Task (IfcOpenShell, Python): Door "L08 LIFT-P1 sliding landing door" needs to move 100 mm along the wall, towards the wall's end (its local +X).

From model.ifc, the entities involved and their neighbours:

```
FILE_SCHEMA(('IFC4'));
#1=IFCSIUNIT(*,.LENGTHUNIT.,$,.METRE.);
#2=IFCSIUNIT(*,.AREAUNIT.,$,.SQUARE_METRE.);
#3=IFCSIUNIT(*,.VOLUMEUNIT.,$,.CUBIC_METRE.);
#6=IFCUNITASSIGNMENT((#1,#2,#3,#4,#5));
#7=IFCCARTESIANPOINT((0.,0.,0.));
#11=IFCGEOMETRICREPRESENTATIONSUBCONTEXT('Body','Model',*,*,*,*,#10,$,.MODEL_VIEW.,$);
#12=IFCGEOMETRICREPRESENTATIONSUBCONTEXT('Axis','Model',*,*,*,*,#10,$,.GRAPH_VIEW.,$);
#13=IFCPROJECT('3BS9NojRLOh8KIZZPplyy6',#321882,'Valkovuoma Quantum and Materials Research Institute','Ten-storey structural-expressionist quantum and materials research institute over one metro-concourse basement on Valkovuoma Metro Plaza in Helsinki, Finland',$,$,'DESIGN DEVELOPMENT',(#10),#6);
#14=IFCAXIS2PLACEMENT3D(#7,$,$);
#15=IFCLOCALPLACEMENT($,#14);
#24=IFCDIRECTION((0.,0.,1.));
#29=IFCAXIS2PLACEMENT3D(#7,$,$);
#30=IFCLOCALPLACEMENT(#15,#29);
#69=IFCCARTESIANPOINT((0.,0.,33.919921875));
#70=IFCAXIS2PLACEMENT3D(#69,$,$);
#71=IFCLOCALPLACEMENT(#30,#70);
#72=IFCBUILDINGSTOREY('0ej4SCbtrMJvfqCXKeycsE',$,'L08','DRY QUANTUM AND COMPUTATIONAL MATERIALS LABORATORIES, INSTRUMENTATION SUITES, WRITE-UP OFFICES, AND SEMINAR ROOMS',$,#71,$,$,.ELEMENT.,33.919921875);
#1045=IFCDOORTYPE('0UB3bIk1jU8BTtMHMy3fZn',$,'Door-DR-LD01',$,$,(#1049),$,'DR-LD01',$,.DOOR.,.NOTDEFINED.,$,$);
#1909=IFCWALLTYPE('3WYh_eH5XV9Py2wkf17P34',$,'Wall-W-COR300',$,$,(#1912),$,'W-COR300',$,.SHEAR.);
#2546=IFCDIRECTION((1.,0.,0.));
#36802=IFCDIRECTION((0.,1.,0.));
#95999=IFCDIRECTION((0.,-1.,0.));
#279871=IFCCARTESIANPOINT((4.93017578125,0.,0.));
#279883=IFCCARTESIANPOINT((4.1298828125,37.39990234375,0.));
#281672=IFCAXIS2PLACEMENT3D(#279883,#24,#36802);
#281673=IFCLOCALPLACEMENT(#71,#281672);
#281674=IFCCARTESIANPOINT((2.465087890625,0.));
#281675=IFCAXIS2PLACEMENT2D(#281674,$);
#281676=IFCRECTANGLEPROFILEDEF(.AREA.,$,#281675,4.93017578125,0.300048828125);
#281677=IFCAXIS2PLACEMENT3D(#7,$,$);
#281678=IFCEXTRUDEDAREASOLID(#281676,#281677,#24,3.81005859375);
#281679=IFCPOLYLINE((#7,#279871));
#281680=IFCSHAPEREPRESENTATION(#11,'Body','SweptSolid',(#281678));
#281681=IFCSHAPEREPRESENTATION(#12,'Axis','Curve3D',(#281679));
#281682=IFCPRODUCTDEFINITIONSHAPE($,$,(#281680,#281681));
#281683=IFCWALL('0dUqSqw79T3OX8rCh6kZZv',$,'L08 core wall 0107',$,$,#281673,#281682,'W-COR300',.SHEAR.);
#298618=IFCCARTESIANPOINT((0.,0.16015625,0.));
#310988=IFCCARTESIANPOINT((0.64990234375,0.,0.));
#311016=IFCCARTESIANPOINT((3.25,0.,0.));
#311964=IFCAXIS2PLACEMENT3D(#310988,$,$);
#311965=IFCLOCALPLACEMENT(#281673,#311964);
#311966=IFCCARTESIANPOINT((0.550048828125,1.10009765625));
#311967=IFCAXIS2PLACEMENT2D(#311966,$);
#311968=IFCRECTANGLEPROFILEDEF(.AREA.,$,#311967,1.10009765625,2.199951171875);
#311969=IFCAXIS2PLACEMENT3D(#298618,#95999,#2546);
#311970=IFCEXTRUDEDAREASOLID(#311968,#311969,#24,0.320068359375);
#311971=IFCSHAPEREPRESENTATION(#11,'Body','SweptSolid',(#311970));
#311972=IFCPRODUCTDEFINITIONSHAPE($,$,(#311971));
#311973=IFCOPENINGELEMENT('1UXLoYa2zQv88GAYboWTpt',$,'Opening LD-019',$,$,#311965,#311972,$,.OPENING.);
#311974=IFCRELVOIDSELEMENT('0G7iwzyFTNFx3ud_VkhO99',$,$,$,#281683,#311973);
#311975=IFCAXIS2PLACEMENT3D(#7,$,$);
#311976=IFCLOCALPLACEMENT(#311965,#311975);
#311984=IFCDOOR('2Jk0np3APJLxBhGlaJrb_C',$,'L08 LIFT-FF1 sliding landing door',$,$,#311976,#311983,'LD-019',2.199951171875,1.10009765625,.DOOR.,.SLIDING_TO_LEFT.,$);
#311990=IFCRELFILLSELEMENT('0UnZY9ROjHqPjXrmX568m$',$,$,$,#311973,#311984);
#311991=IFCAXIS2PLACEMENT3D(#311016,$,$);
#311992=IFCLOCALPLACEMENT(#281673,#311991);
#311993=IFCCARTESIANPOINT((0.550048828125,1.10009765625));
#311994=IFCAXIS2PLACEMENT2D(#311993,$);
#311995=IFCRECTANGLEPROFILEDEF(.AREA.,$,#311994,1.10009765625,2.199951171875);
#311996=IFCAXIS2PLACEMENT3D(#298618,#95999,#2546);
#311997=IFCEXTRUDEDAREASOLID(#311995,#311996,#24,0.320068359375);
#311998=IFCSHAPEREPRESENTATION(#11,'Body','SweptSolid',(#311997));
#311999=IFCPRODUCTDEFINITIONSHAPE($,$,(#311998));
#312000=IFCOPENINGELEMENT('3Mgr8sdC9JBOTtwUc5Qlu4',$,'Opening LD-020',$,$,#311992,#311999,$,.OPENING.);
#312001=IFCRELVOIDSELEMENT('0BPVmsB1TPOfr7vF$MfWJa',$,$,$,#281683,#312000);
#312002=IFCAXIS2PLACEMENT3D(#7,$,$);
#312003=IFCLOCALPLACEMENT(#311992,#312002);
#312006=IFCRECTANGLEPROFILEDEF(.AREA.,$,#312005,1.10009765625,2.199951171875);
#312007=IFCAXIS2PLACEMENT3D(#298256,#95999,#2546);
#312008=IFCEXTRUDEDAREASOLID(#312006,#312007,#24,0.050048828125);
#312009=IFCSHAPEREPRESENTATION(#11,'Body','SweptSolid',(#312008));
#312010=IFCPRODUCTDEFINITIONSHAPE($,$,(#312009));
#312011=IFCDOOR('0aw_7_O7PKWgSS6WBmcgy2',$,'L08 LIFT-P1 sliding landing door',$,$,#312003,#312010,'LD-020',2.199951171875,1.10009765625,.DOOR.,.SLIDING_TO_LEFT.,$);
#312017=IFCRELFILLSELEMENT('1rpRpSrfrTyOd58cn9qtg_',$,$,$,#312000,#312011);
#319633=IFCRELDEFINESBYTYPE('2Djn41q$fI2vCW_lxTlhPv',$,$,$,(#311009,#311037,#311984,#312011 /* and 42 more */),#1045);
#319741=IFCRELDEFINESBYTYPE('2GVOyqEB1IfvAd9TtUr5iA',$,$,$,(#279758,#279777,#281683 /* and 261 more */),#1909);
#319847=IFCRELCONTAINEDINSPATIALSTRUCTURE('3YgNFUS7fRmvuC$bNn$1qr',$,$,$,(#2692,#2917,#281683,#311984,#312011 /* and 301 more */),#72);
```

```python
import ifcopenshell
import ifcopenshell.api.geometry
import ifcopenshell.util.placement

model = ifcopenshell.open("model.ifc")

door = model.by_guid("0aw_7_O7PKWgSS6WBmcgy2")
opening = door.FillsVoids[0].RelatingOpeningElement
wall = opening.VoidsElements[0].RelatingBuildingElement

wall_matrix = ifcopenshell.util.placement.get_local_placement(wall.ObjectPlacement)
shift = wall_matrix[:3, 0] * 0.1
before = ifcopenshell.util.placement.get_local_placement(door.ObjectPlacement)[:3, 3].copy()

# The door is placed relative to its opening, so it follows when the opening moves.
matrix = ifcopenshell.util.placement.get_local_placement(opening.ObjectPlacement)
matrix[:3, 3] += shift
ifcopenshell.api.geometry.edit_object_placement(
    model, product=opening, matrix=matrix, is_si=False, should_transform_children=True
)

after = ifcopenshell.util.placement.get_local_placement(door.ObjectPlacement)[:3, 3]
print("door moved by", (after - before).round(3) + 0.0)

model.write("model_updated.ifc")
```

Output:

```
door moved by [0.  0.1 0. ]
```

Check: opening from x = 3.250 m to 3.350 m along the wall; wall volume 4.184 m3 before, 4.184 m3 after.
